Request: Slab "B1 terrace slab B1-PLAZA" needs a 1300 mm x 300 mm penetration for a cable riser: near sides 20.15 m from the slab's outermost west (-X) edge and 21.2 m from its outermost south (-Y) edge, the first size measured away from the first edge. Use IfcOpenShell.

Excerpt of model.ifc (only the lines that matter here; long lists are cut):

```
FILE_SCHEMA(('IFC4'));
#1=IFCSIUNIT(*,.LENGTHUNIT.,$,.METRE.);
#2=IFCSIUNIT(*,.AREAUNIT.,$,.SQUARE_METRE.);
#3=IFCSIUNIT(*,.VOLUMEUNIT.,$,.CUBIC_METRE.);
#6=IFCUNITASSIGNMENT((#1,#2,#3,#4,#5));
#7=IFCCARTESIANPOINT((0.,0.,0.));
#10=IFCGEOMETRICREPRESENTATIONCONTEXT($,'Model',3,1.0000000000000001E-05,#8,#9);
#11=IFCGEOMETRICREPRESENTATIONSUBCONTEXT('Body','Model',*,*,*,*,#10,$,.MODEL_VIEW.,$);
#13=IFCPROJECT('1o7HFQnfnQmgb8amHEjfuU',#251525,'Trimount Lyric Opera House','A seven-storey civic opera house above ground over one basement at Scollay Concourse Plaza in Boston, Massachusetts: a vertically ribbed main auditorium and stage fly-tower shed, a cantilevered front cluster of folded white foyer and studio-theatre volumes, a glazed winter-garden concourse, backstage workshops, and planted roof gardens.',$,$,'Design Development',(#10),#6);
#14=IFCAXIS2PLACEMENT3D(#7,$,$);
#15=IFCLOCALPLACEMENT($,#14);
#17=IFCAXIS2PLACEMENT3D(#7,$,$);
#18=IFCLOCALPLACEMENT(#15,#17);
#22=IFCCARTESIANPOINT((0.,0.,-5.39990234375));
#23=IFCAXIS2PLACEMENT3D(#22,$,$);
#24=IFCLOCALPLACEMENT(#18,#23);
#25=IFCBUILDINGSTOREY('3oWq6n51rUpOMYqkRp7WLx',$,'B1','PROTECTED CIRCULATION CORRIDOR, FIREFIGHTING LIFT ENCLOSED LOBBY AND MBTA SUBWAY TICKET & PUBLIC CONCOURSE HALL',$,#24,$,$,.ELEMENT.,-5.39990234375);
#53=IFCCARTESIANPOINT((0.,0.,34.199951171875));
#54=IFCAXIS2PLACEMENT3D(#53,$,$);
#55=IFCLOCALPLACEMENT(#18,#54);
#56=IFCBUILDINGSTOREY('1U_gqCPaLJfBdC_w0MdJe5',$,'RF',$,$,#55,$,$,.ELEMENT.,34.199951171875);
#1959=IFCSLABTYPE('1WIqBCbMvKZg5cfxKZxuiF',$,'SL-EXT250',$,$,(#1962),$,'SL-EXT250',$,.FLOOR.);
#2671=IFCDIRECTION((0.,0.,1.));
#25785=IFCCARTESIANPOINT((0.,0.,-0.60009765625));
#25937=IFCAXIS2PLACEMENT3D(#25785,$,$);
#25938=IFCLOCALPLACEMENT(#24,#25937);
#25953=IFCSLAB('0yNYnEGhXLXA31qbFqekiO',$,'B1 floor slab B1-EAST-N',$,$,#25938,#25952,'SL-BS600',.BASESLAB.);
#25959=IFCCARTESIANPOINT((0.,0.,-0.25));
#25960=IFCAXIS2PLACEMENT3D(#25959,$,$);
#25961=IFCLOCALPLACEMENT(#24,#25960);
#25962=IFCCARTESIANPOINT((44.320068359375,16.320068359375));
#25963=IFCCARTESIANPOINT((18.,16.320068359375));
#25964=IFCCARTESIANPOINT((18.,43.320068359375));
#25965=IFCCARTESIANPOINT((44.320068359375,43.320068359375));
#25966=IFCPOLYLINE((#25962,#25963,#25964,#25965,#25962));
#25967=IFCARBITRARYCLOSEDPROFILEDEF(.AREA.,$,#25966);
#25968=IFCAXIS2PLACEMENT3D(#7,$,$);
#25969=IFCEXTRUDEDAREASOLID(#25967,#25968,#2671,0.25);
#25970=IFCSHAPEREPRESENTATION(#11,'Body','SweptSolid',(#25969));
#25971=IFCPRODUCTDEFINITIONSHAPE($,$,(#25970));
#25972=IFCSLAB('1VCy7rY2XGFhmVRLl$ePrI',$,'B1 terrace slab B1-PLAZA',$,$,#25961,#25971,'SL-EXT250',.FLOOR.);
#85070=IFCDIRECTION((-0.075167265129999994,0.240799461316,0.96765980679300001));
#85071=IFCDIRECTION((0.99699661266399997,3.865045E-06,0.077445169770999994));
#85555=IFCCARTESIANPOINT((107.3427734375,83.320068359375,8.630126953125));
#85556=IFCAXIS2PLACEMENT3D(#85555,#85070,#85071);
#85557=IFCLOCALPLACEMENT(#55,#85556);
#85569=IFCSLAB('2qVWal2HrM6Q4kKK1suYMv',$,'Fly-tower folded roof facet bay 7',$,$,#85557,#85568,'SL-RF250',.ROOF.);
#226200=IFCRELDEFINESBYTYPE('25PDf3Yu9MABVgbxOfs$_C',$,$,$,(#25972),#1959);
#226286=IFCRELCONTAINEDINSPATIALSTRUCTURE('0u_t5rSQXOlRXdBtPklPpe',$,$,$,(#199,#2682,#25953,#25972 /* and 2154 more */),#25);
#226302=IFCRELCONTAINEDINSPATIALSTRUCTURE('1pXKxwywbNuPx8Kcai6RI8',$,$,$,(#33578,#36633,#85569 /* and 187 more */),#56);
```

```python
import numpy as np
import ifcopenshell
import ifcopenshell.api.feature
import ifcopenshell.api.geometry
import ifcopenshell.api.root
import ifcopenshell.geom
import ifcopenshell.util.placement
import ifcopenshell.util.representation
import ifcopenshell.util.shape
import ifcopenshell.util.unit

model = ifcopenshell.open("model.ifc")
unit_scale = ifcopenshell.util.unit.calculate_unit_scale(model)
settings = ifcopenshell.geom.settings()


def volume(element):
    """Net volume in cubic metres, openings subtracted."""
    shape = ifcopenshell.geom.create_shape(settings, element)
    return ifcopenshell.util.shape.get_volume(shape.geometry)


slab = model.by_guid("1VCy7rY2XGFhmVRLl$ePrI")
before = volume(slab)

# Extent in the slab's own axes, in metres. The edges named are its -X and -Y sides.
slab_shape = ifcopenshell.geom.create_shape(settings, slab)
vertices = ifcopenshell.util.shape.get_vertices(slab_shape.geometry)
x_min, y_min, bottom = vertices.min(axis=0)
top = vertices[:, 2].max()

opening = ifcopenshell.api.root.create_entity(model, ifc_class="IfcOpeningElement", name="Cable riser opening", predefined_type="OPENING")
context = ifcopenshell.util.representation.get_context(model, "Model", "Body", "MODEL_VIEW")
width, depth = 1.3, 0.3
outline = [(0.0, 0.0), (width, 0.0), (width, depth), (0.0, depth), (0.0, 0.0)]
# Overshoot both faces by 50 mm so the cut is clean.
shape = ifcopenshell.api.geometry.add_slab_representation(
    model, context=context, depth=top - bottom + 0.1, polyline=outline
)
ifcopenshell.api.geometry.assign_representation(model, product=opening, representation=shape)

matrix = ifcopenshell.util.placement.get_local_placement(slab.ObjectPlacement)
matrix[:, 3] = matrix @ np.append(np.array([x_min + 20.15, y_min + 21.2, bottom - 0.05]) / unit_scale, 1.0)
ifcopenshell.api.geometry.edit_object_placement(model, product=opening, matrix=matrix, is_si=False)
ifcopenshell.api.feature.add_feature(model, feature=opening, element=slab)

after = volume(slab)

print(f"slab volume {before:.3f} -> {after:.3f} m3")

model.write("model_rev.ifc")
```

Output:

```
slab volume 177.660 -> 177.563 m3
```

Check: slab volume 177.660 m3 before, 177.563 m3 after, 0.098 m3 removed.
